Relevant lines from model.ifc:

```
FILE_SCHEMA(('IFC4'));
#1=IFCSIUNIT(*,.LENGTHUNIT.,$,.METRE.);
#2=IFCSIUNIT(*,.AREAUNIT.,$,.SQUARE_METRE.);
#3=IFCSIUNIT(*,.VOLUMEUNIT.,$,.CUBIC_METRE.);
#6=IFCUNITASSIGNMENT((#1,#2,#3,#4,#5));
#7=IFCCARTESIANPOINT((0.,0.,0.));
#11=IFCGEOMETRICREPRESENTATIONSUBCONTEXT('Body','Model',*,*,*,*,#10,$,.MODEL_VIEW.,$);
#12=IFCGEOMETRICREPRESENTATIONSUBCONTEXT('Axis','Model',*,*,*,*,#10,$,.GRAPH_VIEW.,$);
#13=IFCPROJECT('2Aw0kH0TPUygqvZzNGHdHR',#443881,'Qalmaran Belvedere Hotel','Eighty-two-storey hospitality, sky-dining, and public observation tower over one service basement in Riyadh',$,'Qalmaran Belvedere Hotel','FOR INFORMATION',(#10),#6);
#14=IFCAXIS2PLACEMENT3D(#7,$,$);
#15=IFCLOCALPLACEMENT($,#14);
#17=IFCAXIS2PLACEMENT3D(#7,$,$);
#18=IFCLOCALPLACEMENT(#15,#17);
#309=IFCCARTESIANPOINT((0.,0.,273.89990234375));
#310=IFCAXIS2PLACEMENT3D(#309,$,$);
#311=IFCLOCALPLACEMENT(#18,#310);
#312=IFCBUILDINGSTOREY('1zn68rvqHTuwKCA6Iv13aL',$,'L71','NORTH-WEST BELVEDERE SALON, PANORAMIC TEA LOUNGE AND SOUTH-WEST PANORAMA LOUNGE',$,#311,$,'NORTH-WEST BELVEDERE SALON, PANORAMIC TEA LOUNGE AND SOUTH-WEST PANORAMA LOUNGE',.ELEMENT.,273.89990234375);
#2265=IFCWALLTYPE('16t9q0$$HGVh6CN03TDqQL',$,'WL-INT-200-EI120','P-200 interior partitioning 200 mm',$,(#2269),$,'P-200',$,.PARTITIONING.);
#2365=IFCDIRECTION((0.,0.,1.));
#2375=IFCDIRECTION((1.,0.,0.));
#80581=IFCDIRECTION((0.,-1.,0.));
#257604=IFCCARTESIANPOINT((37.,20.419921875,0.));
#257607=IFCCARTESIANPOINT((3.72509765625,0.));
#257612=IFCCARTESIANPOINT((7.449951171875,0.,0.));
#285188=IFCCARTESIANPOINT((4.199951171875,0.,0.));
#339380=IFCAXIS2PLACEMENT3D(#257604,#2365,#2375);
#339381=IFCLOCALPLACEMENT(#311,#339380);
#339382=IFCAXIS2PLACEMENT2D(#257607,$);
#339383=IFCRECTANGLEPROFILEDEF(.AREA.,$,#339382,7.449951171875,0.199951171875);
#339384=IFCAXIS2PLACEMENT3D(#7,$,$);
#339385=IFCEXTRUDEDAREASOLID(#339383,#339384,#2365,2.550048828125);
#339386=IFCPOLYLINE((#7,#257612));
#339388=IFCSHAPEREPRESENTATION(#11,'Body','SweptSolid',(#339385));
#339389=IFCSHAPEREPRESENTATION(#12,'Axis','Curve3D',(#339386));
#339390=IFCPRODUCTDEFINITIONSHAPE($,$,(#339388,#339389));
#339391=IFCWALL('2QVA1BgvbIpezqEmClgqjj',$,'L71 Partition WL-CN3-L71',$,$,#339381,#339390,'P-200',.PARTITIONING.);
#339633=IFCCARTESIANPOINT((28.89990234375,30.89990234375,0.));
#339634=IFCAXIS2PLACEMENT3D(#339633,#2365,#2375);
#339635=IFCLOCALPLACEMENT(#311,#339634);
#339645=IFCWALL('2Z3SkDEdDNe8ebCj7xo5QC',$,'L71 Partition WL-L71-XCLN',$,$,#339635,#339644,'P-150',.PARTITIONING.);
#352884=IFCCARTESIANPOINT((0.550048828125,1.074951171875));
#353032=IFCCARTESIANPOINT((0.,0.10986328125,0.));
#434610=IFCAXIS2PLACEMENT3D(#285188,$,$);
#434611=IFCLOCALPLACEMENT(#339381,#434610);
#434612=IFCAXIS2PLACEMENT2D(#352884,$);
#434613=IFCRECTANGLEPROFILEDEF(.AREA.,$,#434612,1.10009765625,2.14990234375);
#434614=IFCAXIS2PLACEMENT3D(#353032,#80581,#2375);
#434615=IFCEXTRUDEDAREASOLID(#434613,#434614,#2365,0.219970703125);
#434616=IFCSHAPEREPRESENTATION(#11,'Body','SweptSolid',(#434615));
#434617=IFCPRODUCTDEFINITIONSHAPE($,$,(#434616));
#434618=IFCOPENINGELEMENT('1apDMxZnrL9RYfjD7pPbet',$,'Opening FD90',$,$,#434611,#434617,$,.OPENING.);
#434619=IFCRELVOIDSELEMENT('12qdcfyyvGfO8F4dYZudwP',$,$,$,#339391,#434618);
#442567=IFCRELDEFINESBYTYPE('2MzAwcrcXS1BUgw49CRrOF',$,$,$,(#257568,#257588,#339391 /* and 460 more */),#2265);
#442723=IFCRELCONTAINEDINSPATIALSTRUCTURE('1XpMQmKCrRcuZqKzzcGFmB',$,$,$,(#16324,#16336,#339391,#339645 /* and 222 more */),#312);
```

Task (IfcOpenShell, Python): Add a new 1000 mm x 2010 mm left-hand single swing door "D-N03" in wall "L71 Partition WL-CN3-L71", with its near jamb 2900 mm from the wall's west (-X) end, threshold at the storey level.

```python
import numpy as np
import ifcopenshell
import ifcopenshell.api.feature
import ifcopenshell.api.geometry
import ifcopenshell.api.root
import ifcopenshell.api.spatial
import ifcopenshell.geom
import ifcopenshell.util.element
import ifcopenshell.util.placement
import ifcopenshell.util.representation
import ifcopenshell.util.shape
import ifcopenshell.util.unit

model = ifcopenshell.open("model.ifc")
unit_scale = ifcopenshell.util.unit.calculate_unit_scale(model)
settings = ifcopenshell.geom.settings()


def volume(element):
    """Net volume in cubic metres, openings subtracted."""
    shape = ifcopenshell.geom.create_shape(settings, element)
    return ifcopenshell.util.shape.get_volume(shape.geometry)


wall = model.by_guid("2QVA1BgvbIpezqEmClgqjj")
storey = ifcopenshell.util.element.get_container(wall, ifc_class="IfcBuildingStorey")
context = ifcopenshell.util.representation.get_context(model, "Model", "Body", "MODEL_VIEW")
before = volume(wall)

width, height, from_end, sill = 1, 2.01, 2.9, 0.0  # metres

# The wall runs along its own X axis, and the end named is its -X end.
wall_shape = ifcopenshell.geom.create_shape(settings, wall)
x, y, z = ifcopenshell.util.shape.get_vertices(wall_shape.geometry).T
start = x.min() + from_end
face, thickness = float(y.min()), float(y.max() - y.min())
wall_matrix = ifcopenshell.util.placement.get_local_placement(wall.ObjectPlacement)
level = ifcopenshell.util.placement.get_local_placement(storey.ObjectPlacement)[2, 3]


def in_wall(x, y):
    """Placement at x, y metres in the wall's axes, at sill height."""
    matrix = wall_matrix.copy()
    matrix[:, 3] = wall_matrix @ np.array([x / unit_scale, y / unit_scale, 0.0, 1.0])
    matrix[2, 3] = level + sill / unit_scale
    return matrix


# Opening: a box that overshoots both wall faces by 50 mm.
opening = ifcopenshell.api.root.create_entity(model, ifc_class="IfcOpeningElement", predefined_type="OPENING")
box = ifcopenshell.api.geometry.add_wall_representation(
    model, context=context, length=width, height=height, thickness=thickness + 0.1
)
ifcopenshell.api.geometry.assign_representation(model, product=opening, representation=box)
ifcopenshell.api.geometry.edit_object_placement(model, product=opening, matrix=in_wall(start, face - 0.05), is_si=False)
ifcopenshell.api.feature.add_feature(model, feature=opening, element=wall)

door = ifcopenshell.api.root.create_entity(model, ifc_class="IfcDoor", name="D-N03", predefined_type="DOOR")
door.OverallWidth, door.OverallHeight = width / unit_scale, height / unit_scale
door.OperationType = "SINGLE_SWING_LEFT"
body = ifcopenshell.api.geometry.add_door_representation(
    model,
    context=context,
    overall_width=door.OverallWidth,
    overall_height=door.OverallHeight,
    operation_type="SINGLE_SWING_LEFT",
    lining_properties={"LiningDepth": thickness / unit_scale, "ThresholdDepth": thickness / unit_scale},
)
ifcopenshell.api.geometry.assign_representation(model, product=door, representation=body)
ifcopenshell.api.spatial.assign_container(model, products=[door], relating_structure=storey)
ifcopenshell.api.feature.add_filling(model, opening=opening, element=door)

# The lining spans the wall, so the door starts at the wall face.
ifcopenshell.api.geometry.edit_object_placement(model, product=door, matrix=in_wall(start, face), is_si=False)

after = volume(wall)

print(f"wall volume {before:.3f} -> {after:.3f} m3")

model.write("model_edited.ifc")
```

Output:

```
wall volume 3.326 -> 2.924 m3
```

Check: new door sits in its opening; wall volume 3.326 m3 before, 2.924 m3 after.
